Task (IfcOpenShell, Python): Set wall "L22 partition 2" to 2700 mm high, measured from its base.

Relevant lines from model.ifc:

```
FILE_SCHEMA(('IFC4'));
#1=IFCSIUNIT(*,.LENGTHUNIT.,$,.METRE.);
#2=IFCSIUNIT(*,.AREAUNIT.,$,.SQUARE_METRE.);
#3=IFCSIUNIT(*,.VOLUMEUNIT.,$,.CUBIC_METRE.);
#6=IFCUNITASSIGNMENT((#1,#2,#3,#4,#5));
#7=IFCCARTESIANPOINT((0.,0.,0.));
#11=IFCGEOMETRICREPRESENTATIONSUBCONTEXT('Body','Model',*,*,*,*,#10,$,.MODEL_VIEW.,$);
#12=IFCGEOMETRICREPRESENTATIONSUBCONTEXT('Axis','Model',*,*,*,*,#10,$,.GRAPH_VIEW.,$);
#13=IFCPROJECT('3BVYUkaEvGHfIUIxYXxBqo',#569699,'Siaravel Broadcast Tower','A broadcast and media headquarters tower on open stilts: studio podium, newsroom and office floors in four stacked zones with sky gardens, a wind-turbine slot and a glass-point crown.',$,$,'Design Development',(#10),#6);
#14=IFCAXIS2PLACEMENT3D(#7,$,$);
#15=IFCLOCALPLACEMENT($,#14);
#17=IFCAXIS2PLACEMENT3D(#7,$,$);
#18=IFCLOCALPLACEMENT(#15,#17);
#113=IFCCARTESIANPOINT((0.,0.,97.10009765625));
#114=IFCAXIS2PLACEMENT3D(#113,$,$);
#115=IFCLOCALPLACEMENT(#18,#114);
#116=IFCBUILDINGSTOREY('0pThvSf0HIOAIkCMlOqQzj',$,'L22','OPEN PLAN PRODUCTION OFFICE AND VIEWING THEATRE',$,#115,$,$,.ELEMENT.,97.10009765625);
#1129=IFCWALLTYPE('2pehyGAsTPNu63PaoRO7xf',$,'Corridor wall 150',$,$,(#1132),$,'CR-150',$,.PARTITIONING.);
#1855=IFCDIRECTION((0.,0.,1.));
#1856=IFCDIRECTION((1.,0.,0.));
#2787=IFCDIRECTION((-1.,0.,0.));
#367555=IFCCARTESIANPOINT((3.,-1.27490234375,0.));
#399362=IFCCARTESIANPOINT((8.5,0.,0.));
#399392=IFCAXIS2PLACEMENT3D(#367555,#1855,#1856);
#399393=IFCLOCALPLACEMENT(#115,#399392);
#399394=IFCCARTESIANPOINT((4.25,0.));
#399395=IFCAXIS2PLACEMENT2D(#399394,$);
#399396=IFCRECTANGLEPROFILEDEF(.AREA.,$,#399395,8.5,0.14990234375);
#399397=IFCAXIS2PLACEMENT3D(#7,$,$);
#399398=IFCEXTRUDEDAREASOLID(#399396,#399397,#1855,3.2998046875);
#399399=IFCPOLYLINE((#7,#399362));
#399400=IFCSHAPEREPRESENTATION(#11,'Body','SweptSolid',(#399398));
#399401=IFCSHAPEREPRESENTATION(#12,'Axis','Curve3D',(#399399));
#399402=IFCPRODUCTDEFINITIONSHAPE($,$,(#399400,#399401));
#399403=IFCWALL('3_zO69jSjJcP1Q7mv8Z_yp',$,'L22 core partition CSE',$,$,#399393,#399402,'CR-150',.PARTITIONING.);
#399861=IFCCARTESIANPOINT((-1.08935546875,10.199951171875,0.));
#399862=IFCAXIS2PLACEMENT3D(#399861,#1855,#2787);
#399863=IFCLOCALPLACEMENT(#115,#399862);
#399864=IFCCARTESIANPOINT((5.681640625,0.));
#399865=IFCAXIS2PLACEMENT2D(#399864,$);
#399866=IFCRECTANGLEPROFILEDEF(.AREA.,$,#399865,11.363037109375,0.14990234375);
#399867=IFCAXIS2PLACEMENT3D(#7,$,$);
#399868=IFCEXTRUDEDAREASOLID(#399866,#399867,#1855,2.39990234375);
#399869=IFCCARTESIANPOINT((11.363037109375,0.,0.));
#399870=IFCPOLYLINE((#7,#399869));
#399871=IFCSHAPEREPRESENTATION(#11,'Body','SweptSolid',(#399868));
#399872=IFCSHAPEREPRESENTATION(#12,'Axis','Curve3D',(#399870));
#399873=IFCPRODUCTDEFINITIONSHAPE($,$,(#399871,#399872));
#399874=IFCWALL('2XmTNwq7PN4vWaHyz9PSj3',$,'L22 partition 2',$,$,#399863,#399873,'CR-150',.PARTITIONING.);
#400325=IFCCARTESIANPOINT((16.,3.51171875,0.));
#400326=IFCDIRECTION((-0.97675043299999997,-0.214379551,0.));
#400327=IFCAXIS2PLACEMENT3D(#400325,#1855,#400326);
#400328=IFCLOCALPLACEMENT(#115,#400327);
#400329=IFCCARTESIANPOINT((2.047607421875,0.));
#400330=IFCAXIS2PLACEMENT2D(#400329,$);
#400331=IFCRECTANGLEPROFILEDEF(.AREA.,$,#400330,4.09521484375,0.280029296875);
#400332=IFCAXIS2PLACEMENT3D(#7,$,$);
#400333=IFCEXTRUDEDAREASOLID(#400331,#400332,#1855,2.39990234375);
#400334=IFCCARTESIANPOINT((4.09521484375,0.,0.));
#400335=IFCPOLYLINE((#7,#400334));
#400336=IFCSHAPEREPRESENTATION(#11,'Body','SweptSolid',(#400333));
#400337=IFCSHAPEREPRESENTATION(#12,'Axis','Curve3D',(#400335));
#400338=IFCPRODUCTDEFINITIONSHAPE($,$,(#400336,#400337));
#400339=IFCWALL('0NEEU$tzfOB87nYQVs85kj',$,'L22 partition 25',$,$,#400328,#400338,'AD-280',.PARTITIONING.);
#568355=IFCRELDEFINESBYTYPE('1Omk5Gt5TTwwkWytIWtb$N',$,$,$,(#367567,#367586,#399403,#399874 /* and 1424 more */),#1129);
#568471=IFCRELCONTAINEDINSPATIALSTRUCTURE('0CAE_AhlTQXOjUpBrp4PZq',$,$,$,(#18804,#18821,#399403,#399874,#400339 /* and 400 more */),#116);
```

```python
import ifcopenshell
import ifcopenshell.geom
import ifcopenshell.util.representation
import ifcopenshell.util.shape
import ifcopenshell.util.unit

model = ifcopenshell.open("model.ifc")
unit_scale = ifcopenshell.util.unit.calculate_unit_scale(model)
settings = ifcopenshell.geom.settings()


def volume(element):
    """Net volume in cubic metres, openings subtracted."""
    shape = ifcopenshell.geom.create_shape(settings, element)
    return ifcopenshell.util.shape.get_volume(shape.geometry)


wall = model.by_guid("2XmTNwq7PN4vWaHyz9PSj3")
before = volume(wall)

body = ifcopenshell.util.representation.get_representation(wall, "Model", "Body")
solid = body.Items[0]
old_height = solid.Depth
solid.Depth = 2.7 / unit_scale
after = volume(wall)

print(f"height {old_height:g} -> {solid.Depth:g}, volume {before:.3f} -> {after:.3f} m3")

model.write("model_v2.ifc")
```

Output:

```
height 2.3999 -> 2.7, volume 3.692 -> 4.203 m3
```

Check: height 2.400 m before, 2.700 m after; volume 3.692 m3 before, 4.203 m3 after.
